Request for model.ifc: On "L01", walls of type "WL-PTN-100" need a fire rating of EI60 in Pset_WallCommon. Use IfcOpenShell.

First a look at what the model holds.

```python
import ifcopenshell
import ifcopenshell.util.element

model = ifcopenshell.open("model.ifc")
print(model.schema)
storey = next(s for s in model.by_type("IfcBuildingStorey") if s.Name == "L01")
walls = [e for e in ifcopenshell.util.element.get_decomposition(storey) if e.is_a("IfcWall")]
seen = {}
for e in walls:
    element_type = ifcopenshell.util.element.get_type(e)
    key = (element_type.Name if element_type != e and element_type else None, ifcopenshell.util.element.get_pset(e, "Pset_WallCommon", "FireRating"))
    seen[key] = seen.get(key, 0) + 1
for (name, value), count in sorted(seen.items(), key=str):
    print(count, "x", name, "|", value)
```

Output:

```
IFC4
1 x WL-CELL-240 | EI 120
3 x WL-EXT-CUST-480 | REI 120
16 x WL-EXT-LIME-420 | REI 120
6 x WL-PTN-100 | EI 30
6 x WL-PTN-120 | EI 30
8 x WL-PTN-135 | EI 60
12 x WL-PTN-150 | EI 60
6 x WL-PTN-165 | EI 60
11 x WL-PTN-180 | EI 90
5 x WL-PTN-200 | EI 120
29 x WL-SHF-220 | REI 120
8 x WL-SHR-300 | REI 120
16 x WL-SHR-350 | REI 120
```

```python
import ifcopenshell
import ifcopenshell.api.pset
import ifcopenshell.util.element

model = ifcopenshell.open("model.ifc")

storey = next(s for s in model.by_type("IfcBuildingStorey") if s.Name == "L01")
walls = [e for e in ifcopenshell.util.element.get_decomposition(storey) if e.is_a("IfcWall")]

count = 0
for e in walls:
    element_type = ifcopenshell.util.element.get_type(e)
    if element_type in (None, e) or element_type.Name != "WL-PTN-100":
        continue
    # add_pset returns the element's existing set when there is one.
    pset = ifcopenshell.api.pset.add_pset(model, product=e, name="Pset_WallCommon")
    ifcopenshell.api.pset.edit_pset(model, pset=pset, properties={"FireRating": "EI60"})
    count += 1

print(count, "walls updated")

model.write("model_edited.ifc")
```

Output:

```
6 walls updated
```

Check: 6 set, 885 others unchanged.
